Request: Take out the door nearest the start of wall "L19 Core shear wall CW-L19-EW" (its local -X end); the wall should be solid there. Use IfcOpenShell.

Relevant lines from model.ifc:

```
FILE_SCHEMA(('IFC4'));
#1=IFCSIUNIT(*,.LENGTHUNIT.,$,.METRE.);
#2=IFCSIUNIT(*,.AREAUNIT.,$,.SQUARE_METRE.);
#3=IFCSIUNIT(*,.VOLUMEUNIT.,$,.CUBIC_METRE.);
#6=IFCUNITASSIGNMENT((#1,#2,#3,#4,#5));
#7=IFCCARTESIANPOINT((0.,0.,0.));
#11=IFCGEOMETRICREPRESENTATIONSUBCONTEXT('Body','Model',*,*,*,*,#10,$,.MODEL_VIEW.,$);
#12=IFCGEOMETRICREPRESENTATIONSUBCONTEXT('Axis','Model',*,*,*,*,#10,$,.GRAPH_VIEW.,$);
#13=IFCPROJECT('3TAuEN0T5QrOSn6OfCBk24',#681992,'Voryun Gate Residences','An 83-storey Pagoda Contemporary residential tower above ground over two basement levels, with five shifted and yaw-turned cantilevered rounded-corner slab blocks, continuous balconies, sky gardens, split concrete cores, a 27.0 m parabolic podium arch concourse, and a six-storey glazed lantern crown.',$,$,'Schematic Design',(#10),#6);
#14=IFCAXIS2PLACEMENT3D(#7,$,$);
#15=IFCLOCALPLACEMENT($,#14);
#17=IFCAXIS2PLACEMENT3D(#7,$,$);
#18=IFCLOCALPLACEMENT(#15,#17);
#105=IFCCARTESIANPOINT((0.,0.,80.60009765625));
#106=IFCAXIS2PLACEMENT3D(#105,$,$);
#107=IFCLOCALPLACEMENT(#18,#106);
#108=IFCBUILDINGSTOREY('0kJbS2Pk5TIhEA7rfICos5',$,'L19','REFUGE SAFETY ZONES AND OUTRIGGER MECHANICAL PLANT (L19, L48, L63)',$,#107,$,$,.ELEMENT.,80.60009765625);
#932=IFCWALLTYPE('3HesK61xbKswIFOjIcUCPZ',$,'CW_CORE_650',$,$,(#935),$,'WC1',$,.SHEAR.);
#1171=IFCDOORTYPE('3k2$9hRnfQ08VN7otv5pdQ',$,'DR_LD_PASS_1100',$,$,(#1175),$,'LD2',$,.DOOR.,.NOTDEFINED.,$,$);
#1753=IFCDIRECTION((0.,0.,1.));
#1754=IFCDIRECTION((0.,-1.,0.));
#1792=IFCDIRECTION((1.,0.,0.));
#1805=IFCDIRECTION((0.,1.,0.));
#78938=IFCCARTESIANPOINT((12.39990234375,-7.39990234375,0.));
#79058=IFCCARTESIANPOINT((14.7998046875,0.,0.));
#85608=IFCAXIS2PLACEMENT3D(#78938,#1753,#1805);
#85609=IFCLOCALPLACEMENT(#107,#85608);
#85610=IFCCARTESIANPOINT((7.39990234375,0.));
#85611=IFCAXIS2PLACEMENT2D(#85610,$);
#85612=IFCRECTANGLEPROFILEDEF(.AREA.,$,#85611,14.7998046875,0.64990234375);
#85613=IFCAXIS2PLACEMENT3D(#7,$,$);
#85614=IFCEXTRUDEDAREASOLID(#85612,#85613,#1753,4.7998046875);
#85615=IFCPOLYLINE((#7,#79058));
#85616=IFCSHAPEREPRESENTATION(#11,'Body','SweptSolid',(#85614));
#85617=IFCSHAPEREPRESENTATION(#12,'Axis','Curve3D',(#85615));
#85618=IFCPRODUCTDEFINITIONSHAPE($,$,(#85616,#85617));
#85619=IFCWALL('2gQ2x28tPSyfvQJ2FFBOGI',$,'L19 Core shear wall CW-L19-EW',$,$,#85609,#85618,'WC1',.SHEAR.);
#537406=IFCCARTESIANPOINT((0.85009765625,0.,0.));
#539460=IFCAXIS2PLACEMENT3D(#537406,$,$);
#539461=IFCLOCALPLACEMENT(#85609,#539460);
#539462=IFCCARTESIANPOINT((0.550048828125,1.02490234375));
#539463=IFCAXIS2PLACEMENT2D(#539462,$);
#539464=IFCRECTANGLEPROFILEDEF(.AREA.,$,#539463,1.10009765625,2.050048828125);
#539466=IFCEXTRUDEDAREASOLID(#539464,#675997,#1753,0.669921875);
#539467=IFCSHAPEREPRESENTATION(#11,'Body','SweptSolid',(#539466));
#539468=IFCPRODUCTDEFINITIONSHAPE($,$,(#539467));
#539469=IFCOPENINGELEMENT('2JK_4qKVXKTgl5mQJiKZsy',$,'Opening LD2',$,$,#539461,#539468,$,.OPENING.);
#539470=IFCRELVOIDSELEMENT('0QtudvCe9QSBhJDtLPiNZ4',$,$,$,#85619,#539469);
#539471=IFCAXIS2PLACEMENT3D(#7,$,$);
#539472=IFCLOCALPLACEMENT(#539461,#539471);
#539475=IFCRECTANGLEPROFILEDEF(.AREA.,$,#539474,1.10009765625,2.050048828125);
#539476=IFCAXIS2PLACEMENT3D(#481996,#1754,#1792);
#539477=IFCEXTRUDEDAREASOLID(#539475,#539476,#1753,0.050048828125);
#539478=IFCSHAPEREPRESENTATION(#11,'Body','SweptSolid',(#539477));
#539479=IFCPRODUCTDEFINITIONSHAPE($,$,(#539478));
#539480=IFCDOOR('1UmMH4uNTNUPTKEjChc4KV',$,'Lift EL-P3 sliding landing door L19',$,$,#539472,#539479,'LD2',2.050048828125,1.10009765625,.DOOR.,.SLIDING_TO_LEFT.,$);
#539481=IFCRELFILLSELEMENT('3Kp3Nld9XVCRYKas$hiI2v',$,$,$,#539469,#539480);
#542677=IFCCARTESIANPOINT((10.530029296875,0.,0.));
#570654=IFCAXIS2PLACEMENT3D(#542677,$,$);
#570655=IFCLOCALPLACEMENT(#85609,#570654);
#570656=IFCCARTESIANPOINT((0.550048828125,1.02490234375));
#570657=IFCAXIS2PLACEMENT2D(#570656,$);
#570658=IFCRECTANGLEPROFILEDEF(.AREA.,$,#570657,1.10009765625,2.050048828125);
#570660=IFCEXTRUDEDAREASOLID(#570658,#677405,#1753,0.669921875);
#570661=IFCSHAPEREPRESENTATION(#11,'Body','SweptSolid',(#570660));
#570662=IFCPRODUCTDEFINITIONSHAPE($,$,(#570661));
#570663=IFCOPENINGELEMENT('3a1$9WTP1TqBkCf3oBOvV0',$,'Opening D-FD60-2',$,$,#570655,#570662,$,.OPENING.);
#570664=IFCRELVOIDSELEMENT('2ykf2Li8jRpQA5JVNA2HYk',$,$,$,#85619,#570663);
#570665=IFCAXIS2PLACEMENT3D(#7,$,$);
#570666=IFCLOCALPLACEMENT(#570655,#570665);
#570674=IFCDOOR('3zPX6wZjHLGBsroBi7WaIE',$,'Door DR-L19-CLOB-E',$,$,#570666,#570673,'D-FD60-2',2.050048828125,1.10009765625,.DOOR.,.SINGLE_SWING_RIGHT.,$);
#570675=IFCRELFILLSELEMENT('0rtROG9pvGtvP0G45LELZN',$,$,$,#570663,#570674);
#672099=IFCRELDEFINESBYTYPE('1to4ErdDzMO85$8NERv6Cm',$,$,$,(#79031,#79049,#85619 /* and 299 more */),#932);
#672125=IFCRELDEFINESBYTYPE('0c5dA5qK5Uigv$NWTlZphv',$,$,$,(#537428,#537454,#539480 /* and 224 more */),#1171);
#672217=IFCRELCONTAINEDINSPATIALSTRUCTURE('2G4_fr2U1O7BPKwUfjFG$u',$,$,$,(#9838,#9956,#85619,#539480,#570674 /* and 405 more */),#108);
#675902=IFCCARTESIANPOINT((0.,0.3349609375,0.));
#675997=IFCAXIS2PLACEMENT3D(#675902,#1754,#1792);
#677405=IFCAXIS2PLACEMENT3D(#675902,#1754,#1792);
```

```python
import ifcopenshell
import ifcopenshell.api.feature
import ifcopenshell.api.root
import ifcopenshell.geom
import ifcopenshell.util.shape

model = ifcopenshell.open("model.ifc")
settings = ifcopenshell.geom.settings()


def volume(element):
    """Net volume in cubic metres, openings subtracted."""
    shape = ifcopenshell.geom.create_shape(settings, element)
    return ifcopenshell.util.shape.get_volume(shape.geometry)


door = model.by_guid("1UmMH4uNTNUPTKEjChc4KV")
opening = door.FillsVoids[0].RelatingOpeningElement
wall = opening.VoidsElements[0].RelatingBuildingElement
before = volume(wall)

ifcopenshell.api.root.remove_product(model, product=door)
ifcopenshell.api.feature.remove_feature(model, feature=opening)

after = volume(wall)

print(f"wall volume {before:.3f} -> {after:.3f} m3")

model.write("model_updated.ifc")
```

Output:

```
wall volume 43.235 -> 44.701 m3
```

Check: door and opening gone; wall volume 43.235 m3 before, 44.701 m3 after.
